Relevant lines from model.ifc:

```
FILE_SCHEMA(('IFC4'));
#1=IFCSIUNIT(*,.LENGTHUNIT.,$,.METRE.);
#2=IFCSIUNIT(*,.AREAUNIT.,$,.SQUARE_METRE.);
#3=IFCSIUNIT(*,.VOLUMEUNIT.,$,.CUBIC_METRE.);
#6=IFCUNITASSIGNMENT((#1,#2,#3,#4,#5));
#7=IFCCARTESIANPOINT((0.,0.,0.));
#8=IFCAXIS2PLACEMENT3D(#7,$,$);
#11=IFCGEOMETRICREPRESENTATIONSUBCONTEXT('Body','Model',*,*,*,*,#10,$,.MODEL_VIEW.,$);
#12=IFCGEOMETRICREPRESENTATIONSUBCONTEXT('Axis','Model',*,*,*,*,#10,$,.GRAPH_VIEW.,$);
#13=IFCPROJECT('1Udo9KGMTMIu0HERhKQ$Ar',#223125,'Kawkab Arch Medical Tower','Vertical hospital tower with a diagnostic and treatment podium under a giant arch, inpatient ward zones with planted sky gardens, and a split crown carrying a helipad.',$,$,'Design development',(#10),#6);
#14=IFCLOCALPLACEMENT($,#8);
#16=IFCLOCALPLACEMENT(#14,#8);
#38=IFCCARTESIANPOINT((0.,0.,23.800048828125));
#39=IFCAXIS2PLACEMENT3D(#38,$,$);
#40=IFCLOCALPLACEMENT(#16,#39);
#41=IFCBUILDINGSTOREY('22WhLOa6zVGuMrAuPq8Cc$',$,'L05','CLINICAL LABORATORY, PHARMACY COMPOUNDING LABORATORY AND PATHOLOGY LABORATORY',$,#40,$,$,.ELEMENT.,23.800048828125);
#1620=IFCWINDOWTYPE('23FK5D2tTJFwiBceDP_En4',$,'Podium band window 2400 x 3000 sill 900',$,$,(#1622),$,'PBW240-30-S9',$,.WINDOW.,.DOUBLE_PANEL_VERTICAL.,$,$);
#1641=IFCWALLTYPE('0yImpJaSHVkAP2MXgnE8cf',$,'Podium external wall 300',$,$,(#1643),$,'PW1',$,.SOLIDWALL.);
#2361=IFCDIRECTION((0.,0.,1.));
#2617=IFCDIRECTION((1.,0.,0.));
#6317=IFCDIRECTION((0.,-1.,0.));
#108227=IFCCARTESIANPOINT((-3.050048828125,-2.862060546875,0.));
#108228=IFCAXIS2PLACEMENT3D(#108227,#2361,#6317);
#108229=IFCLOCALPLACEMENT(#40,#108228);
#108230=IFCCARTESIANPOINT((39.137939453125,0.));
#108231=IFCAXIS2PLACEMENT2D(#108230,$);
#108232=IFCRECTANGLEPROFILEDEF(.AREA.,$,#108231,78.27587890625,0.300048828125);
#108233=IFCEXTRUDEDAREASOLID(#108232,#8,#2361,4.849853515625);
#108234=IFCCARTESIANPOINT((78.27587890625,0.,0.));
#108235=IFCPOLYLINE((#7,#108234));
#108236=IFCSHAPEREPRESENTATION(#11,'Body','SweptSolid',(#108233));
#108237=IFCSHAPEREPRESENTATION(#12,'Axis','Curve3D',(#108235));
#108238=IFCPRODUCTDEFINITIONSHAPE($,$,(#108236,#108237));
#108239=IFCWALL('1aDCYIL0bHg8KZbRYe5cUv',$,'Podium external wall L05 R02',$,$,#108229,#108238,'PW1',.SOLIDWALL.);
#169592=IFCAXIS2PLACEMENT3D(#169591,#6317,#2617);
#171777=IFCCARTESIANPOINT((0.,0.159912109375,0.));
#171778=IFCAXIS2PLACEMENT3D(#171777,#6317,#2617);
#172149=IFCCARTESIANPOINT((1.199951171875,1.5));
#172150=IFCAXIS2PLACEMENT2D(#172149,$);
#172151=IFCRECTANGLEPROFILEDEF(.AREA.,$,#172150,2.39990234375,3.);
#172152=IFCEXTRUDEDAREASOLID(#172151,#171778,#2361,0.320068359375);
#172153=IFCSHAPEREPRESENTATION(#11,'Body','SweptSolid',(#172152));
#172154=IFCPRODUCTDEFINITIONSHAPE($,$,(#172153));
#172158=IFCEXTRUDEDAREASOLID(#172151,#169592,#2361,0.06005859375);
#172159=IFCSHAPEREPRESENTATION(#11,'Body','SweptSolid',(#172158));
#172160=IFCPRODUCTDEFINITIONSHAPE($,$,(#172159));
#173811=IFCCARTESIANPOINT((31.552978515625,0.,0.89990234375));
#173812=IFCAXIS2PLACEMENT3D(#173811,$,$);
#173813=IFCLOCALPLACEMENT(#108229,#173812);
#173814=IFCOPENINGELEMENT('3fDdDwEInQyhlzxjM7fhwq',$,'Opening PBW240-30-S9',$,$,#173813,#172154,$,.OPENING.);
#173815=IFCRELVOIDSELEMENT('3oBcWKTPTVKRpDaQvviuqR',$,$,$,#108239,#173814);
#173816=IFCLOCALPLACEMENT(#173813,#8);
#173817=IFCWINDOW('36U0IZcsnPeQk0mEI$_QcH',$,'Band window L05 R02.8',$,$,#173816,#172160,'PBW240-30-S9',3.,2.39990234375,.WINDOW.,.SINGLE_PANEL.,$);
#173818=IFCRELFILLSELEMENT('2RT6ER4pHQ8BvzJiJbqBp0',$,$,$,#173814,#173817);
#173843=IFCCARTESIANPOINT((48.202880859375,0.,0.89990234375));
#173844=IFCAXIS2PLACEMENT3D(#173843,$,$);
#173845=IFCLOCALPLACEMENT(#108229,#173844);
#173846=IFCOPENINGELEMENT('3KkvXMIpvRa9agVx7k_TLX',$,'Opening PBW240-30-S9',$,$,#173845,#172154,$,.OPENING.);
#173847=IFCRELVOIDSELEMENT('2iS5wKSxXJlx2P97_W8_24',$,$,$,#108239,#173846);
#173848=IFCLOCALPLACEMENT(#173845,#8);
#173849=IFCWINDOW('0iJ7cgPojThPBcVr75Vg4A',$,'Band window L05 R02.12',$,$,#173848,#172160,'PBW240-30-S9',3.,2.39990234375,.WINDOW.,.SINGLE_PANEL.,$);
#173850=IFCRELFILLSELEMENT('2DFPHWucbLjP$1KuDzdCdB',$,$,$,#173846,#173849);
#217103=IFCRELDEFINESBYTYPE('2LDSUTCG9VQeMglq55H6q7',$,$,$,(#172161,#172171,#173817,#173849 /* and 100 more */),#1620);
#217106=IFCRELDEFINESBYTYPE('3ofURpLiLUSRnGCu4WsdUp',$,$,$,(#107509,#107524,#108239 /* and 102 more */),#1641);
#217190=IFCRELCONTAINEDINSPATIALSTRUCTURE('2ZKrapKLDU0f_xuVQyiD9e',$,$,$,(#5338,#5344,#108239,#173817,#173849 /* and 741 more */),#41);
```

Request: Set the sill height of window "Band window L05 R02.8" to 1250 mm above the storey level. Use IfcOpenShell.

```python
import numpy as np
import ifcopenshell
import ifcopenshell.api.geometry
import ifcopenshell.geom
import ifcopenshell.util.element
import ifcopenshell.util.placement
import ifcopenshell.util.shape
import ifcopenshell.util.unit

model = ifcopenshell.open("model.ifc")
unit_scale = ifcopenshell.util.unit.calculate_unit_scale(model)

window = model.by_guid("36U0IZcsnPeQk0mEI$_QcH")
opening = window.FillsVoids[0].RelatingOpeningElement
storey = ifcopenshell.util.element.get_container(window, ifc_class="IfcBuildingStorey")
level = ifcopenshell.util.placement.get_local_placement(storey.ObjectPlacement)[2, 3]

# The opening's origin need not be at the sill, so measure its lowest point.
shape = ifcopenshell.geom.create_shape(ifcopenshell.geom.settings(), opening)
bottom = ifcopenshell.util.shape.get_shape_bottom_elevation(shape, shape.geometry) / unit_scale
dz = level + 1.25 / unit_scale - bottom

shift = np.array([0.0, 0.0, dz])
# The window is placed relative to its opening, so it follows when the opening moves.
matrix = ifcopenshell.util.placement.get_local_placement(opening.ObjectPlacement)
matrix[:3, 3] += shift
ifcopenshell.api.geometry.edit_object_placement(
    model, product=opening, matrix=matrix, is_si=False, should_transform_children=True
)

print(f"moved by {dz * unit_scale:+.3f} m")

model.write("model_rev.ifc")
```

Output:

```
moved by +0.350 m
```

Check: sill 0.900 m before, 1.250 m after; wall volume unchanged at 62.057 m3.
